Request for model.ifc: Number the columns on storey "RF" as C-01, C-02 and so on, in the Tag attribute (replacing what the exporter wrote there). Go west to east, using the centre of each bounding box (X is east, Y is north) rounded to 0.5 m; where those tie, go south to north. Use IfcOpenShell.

First a look at what the model holds.

```python
import ifcopenshell
import ifcopenshell.util.element
import ifcopenshell.util.placement

model = ifcopenshell.open("model.ifc")
print(model.schema)
storey = next(s for s in model.by_type("IfcBuildingStorey") if s.Name == "RF")
columns = [e for e in ifcopenshell.util.element.get_decomposition(storey) if e.is_a("IfcColumn")]
for e in sorted(columns, key=lambda e: e.id()):
    origin = ifcopenshell.util.placement.get_local_placement(e.ObjectPlacement)[:3, 3]
    print(e.id(), e.Tag, e.Name, origin.round(2) + 0.0, sep=" | ")
```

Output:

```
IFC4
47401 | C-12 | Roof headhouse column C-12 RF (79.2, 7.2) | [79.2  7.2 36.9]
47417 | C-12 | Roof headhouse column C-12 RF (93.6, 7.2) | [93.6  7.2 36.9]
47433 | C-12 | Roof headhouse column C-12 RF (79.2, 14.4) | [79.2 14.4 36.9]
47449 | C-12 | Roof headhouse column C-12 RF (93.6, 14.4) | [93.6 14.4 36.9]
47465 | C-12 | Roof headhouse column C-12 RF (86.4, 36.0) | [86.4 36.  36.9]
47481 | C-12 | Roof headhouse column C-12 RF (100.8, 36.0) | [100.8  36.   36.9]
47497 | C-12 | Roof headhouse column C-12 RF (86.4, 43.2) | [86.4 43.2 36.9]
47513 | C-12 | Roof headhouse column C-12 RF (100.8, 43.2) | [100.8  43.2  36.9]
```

```python
import ifcopenshell
import ifcopenshell.geom
import ifcopenshell.util.element
import ifcopenshell.util.shape

model = ifcopenshell.open("model.ifc")
settings = ifcopenshell.geom.settings()
settings.set("use-world-coords", True)


def centre(element):
    shape = ifcopenshell.geom.create_shape(settings, element)
    return ifcopenshell.util.shape.get_bbox_centroid(shape.geometry)


storey = next(s for s in model.by_type("IfcBuildingStorey") if s.Name == "RF")
columns = [e for e in ifcopenshell.util.element.get_decomposition(storey) if e.is_a("IfcColumn")]

# Insertion points can sit at a corner or the storey origin, so sort by the geometry (in metres).
centres = {e: centre(e) for e in columns}
columns.sort(key=lambda e: (round(centres[e][0] / 0.5), centres[e][1]))

for i, e in enumerate(columns, start=1):
    number = f"C-{i:02d}"
    e.Tag = number
    print(e.id(), number)

model.write("model_rev.ifc")
```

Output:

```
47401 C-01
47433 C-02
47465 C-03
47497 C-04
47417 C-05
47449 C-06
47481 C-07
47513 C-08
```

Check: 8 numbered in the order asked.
